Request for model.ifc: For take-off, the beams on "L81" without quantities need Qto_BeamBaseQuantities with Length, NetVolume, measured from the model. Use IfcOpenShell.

First a look at what the model holds.

```python
import ifcopenshell
import ifcopenshell.util.element
import ifcopenshell.util.unit

model = ifcopenshell.open("model.ifc")
print(model.schema)
for unit_type in ("LENGTHUNIT", "AREAUNIT", "VOLUMEUNIT"):
    print(unit_type, ifcopenshell.util.unit.calculate_unit_scale(model, unit_type))
storey = next(s for s in model.by_type("IfcBuildingStorey") if s.Name == "L81")
beams = [e for e in ifcopenshell.util.element.get_decomposition(storey) if e.is_a("IfcBeam")]
for e in sorted(beams, key=lambda e: e.id()):
    print(e.id(), e.is_a(), e.Name, list(ifcopenshell.util.element.get_psets(e, qtos_only=True)), sep=" | ")
```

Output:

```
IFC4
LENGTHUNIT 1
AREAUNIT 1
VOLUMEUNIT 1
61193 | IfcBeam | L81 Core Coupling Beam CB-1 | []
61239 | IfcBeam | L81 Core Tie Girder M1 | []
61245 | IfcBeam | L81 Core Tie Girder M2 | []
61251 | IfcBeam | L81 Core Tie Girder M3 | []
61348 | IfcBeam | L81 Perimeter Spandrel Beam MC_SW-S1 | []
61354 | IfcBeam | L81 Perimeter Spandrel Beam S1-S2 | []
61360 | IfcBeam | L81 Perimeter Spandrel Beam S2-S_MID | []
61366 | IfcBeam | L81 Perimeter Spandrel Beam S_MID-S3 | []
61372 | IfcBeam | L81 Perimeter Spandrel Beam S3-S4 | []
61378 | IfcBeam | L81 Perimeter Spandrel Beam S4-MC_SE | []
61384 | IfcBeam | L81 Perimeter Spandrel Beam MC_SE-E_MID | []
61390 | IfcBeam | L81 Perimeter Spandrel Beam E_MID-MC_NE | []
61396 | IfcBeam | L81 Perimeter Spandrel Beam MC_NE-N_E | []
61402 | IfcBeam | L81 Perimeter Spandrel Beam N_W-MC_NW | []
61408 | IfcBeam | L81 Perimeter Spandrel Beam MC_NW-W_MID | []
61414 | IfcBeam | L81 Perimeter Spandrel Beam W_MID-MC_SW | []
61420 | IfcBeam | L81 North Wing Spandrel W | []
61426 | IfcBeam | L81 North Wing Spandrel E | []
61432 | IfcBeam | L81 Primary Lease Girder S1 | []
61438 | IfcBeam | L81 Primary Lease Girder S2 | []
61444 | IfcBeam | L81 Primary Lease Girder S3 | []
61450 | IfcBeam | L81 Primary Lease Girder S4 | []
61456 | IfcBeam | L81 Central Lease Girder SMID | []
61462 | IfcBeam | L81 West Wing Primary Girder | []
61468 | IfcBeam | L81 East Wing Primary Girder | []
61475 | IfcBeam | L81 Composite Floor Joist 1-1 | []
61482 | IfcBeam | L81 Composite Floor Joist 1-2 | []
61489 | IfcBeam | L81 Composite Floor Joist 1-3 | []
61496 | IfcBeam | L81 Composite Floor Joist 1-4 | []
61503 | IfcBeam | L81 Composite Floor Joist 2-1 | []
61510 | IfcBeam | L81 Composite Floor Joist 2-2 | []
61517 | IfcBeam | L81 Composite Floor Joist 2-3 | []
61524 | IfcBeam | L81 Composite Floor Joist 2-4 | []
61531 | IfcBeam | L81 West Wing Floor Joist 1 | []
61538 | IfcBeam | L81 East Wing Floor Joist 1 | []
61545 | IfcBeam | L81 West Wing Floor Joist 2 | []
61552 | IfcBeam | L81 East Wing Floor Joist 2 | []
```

```python
import ifcopenshell
import ifcopenshell.api.pset
import ifcopenshell.geom
import ifcopenshell.util.element
import ifcopenshell.util.shape
import ifcopenshell.util.unit

model = ifcopenshell.open("model.ifc")
unit_scale = ifcopenshell.util.unit.calculate_unit_scale(model)
volume_scale = ifcopenshell.util.unit.calculate_unit_scale(model, "VOLUMEUNIT")
settings = ifcopenshell.geom.settings()

storey = next(s for s in model.by_type("IfcBuildingStorey") if s.Name == "L81")
beams = [e for e in ifcopenshell.util.element.get_decomposition(storey) if e.is_a("IfcBeam")]

for e in sorted(beams, key=lambda e: e.id()):
    if ifcopenshell.util.element.get_psets(e, qtos_only=True, should_inherit=False):
        continue
    # Geometry comes back in metres, in the element's own axes.
    shape = ifcopenshell.geom.create_shape(settings, e)
    values = {
        "Length": ifcopenshell.util.shape.get_max_xyz(shape.geometry) / unit_scale,
        "NetVolume": ifcopenshell.util.shape.get_volume(shape.geometry) / volume_scale,
    }
    qto = ifcopenshell.api.pset.add_qto(model, product=e, name="Qto_BeamBaseQuantities")
    ifcopenshell.api.pset.edit_qto(model, qto=qto, properties=values)
    print(e.id(), {k: round(v, 3) for k, v in values.items()})

model.write("model-out.ifc")
```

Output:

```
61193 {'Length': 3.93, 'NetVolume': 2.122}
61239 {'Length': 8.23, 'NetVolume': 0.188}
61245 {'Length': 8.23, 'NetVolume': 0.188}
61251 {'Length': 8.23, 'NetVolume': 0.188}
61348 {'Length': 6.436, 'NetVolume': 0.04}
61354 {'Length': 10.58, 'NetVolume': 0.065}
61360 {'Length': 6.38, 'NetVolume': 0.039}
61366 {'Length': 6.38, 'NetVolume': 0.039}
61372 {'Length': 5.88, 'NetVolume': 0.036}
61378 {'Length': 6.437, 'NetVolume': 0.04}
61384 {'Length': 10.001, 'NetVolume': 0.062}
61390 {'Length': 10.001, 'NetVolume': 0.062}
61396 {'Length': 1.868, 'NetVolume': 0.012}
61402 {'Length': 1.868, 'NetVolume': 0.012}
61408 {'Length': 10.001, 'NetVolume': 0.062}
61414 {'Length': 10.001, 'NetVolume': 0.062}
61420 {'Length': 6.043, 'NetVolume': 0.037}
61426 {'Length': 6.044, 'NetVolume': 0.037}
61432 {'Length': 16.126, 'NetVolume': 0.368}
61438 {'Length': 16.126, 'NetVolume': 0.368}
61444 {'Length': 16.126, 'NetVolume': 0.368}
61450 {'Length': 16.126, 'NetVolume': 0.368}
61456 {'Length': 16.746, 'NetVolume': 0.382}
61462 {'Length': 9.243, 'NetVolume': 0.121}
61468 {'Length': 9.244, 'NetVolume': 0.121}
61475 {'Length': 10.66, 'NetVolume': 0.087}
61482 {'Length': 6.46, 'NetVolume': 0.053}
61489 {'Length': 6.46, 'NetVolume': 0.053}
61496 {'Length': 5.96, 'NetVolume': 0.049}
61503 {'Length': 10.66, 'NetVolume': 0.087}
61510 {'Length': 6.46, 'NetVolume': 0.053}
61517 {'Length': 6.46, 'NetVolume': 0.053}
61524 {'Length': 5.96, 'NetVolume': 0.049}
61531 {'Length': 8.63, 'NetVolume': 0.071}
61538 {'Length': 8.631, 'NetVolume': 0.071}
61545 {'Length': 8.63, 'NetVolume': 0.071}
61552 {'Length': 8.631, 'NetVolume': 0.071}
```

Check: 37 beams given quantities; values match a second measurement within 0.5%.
